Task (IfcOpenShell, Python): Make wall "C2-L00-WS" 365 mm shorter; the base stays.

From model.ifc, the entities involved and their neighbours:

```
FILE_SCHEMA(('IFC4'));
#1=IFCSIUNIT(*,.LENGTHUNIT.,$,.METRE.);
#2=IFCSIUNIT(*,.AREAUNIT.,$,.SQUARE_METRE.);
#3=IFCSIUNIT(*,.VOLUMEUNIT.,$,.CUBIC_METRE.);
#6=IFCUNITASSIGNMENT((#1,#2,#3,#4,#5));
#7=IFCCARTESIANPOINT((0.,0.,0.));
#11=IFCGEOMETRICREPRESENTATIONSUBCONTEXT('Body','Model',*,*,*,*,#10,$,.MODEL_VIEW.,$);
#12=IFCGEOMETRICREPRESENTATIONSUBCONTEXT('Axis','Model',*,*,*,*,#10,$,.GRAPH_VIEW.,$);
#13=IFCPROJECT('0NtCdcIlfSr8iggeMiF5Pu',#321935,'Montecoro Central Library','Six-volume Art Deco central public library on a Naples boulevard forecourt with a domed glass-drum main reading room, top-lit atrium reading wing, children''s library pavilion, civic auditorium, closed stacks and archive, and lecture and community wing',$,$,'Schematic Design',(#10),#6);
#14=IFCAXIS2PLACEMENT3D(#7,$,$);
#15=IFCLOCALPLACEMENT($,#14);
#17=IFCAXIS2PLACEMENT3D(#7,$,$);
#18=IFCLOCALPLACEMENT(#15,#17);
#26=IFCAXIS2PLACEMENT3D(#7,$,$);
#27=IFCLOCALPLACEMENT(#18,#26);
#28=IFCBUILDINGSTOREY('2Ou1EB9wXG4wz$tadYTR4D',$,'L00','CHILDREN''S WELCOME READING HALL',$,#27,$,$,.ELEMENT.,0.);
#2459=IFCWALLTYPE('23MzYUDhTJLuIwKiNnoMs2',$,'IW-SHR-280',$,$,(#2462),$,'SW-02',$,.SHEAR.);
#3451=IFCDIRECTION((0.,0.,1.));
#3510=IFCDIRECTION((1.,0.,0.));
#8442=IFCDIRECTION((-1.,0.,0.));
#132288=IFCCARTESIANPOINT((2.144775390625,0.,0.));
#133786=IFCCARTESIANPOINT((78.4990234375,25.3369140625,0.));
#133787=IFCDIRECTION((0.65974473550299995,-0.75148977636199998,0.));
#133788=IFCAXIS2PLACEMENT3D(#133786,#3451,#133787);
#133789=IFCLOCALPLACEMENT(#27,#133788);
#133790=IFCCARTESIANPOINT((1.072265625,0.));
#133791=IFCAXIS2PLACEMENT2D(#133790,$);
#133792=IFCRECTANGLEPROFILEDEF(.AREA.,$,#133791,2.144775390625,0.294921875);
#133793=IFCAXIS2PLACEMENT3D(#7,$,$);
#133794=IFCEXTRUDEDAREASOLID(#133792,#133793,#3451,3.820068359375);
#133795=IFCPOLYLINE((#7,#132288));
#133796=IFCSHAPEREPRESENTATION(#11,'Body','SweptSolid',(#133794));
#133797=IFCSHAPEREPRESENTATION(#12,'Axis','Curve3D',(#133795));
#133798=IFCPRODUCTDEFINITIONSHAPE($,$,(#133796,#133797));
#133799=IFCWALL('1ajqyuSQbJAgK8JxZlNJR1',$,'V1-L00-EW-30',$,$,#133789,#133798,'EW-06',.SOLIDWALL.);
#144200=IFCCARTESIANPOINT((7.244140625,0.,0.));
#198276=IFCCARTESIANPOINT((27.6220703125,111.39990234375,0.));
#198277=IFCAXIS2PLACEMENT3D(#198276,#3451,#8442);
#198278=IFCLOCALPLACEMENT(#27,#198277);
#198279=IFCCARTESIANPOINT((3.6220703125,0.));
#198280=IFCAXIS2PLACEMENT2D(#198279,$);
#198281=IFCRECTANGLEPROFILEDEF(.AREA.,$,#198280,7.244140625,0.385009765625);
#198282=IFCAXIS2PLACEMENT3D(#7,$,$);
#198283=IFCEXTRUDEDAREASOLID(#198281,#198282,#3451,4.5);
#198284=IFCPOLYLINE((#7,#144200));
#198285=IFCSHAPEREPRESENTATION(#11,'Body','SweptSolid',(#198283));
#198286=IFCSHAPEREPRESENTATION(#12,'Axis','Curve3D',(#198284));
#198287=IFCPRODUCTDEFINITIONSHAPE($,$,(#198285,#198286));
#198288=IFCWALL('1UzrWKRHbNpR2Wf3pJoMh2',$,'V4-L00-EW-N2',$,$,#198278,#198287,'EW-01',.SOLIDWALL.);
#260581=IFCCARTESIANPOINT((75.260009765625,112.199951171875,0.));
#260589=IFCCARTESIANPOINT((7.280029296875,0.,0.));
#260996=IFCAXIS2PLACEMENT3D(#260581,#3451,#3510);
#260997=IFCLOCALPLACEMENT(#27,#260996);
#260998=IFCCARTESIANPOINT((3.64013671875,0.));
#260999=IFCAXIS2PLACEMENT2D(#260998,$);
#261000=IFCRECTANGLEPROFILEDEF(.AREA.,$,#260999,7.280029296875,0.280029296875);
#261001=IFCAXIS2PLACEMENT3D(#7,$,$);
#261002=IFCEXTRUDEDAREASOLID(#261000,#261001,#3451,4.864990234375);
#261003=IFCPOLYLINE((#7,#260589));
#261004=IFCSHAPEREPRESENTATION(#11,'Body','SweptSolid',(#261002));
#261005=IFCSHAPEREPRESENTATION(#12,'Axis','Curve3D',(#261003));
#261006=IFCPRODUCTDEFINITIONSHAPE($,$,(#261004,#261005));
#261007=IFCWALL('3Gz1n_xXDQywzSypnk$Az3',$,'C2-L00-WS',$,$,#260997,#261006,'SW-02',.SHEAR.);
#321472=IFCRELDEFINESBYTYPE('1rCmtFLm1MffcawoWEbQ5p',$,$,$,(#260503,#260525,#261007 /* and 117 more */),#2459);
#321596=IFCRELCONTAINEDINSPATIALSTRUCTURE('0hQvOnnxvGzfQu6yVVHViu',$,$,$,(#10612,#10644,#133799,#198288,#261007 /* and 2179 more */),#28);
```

```python
import ifcopenshell
import ifcopenshell.geom
import ifcopenshell.util.representation
import ifcopenshell.util.shape
import ifcopenshell.util.unit

model = ifcopenshell.open("model.ifc")
unit_scale = ifcopenshell.util.unit.calculate_unit_scale(model)
settings = ifcopenshell.geom.settings()


def volume(element):
    """Net volume in cubic metres, openings subtracted."""
    shape = ifcopenshell.geom.create_shape(settings, element)
    return ifcopenshell.util.shape.get_volume(shape.geometry)


wall = model.by_id(261007)
before = volume(wall)

body = ifcopenshell.util.representation.get_representation(wall, "Model", "Body")
solid = body.Items[0]
old_height = solid.Depth
solid.Depth -= 0.365 / unit_scale
after = volume(wall)

print(f"height {old_height:g} -> {solid.Depth:g}, volume {before:.3f} -> {after:.3f} m3")

model.write("model_rev.ifc")
```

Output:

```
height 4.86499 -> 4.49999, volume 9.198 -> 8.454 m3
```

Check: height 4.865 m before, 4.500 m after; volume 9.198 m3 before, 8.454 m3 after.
